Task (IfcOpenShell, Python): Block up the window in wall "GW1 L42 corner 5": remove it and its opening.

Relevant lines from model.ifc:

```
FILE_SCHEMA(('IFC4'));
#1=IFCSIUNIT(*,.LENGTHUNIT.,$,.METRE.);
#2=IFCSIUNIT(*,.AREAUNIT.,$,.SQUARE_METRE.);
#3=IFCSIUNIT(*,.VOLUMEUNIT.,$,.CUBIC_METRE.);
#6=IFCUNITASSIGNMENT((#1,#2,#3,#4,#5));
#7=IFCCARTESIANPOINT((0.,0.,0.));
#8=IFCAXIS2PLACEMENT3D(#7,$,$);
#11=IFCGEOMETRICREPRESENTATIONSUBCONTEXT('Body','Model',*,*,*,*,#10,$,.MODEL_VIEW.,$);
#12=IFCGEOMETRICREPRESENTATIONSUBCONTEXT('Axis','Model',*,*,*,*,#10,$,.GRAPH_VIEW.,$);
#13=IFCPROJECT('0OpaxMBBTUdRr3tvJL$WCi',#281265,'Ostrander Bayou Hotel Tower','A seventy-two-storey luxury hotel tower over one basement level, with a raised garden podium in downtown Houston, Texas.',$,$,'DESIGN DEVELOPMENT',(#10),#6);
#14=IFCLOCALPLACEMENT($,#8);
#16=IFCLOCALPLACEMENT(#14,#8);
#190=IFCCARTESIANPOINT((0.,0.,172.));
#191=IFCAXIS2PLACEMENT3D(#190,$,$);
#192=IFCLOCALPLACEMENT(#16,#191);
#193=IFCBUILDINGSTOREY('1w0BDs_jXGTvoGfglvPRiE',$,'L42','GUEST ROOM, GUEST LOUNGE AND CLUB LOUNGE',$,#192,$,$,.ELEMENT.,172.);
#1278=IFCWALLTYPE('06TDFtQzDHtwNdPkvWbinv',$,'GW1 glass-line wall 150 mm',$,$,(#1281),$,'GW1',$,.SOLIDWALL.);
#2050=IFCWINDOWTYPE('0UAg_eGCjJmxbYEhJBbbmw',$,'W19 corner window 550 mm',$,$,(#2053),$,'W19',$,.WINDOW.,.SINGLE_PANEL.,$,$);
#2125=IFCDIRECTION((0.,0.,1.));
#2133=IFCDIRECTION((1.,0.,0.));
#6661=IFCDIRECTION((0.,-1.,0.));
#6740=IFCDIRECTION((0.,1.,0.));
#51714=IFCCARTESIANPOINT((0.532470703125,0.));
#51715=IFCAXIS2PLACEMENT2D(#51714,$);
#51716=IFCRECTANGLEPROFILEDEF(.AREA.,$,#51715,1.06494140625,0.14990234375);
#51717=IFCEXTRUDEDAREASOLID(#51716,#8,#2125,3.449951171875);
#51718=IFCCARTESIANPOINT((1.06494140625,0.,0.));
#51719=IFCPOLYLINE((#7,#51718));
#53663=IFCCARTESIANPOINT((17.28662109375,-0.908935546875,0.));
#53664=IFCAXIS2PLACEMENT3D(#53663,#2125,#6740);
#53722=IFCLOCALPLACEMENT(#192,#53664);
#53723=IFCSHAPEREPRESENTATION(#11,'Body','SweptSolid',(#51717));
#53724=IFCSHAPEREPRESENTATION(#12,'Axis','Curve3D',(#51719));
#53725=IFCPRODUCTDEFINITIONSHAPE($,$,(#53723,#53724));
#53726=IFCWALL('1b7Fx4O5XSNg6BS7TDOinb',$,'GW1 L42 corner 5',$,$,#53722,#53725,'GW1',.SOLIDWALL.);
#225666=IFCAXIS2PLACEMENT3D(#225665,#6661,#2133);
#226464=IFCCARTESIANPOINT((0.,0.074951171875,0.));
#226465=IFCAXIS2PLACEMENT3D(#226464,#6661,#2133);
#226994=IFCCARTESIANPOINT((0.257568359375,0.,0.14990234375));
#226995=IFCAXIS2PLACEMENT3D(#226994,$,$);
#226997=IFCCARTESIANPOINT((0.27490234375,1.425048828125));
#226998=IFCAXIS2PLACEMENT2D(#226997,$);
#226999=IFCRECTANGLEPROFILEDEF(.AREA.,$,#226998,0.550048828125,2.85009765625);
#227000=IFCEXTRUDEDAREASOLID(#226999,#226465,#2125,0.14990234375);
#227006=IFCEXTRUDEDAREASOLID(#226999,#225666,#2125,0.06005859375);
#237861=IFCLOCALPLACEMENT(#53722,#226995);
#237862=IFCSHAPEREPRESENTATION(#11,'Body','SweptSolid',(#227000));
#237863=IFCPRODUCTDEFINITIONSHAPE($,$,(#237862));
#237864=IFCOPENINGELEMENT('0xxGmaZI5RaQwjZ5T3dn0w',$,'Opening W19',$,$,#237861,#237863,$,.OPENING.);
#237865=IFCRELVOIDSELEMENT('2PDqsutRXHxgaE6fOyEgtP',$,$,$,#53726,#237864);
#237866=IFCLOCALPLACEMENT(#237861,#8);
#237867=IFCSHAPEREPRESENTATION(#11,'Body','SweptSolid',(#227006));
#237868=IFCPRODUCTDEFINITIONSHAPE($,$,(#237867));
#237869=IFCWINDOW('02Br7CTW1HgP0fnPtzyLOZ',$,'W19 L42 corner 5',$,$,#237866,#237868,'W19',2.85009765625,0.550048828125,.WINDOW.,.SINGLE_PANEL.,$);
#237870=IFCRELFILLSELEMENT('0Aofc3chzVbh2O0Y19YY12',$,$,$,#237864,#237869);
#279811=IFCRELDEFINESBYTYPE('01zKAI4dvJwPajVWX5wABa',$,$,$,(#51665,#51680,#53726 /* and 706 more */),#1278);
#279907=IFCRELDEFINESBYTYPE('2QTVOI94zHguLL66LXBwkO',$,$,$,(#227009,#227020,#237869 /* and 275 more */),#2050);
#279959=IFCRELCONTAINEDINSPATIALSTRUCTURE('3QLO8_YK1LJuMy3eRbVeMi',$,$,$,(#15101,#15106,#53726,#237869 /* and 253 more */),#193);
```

```python
import ifcopenshell
import ifcopenshell.api.feature
import ifcopenshell.api.root
import ifcopenshell.geom
import ifcopenshell.util.shape

model = ifcopenshell.open("model.ifc")
settings = ifcopenshell.geom.settings()


def volume(element):
    """Net volume in cubic metres, openings subtracted."""
    shape = ifcopenshell.geom.create_shape(settings, element)
    return ifcopenshell.util.shape.get_volume(shape.geometry)


window = model.by_id(237869)
opening = window.FillsVoids[0].RelatingOpeningElement
wall = opening.VoidsElements[0].RelatingBuildingElement
before = volume(wall)

ifcopenshell.api.root.remove_product(model, product=window)
ifcopenshell.api.feature.remove_feature(model, feature=opening)

after = volume(wall)

print(f"wall volume {before:.3f} -> {after:.3f} m3")

model.write("model_updated.ifc")
```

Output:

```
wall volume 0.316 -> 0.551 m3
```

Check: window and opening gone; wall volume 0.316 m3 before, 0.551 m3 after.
